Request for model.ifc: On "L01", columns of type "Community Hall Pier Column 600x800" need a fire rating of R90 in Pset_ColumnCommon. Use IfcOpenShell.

First a look at what the model holds.

```python
import ifcopenshell
import ifcopenshell.util.element

model = ifcopenshell.open("model.ifc")
print(model.schema)
storey = next(s for s in model.by_type("IfcBuildingStorey") if s.Name == "L01")
columns = [e for e in ifcopenshell.util.element.get_decomposition(storey) if e.is_a("IfcColumn")]
seen = {}
for e in columns:
    element_type = ifcopenshell.util.element.get_type(e)
    key = (element_type.Name if element_type != e and element_type else None, ifcopenshell.util.element.get_pset(e, "Pset_ColumnCommon", "FireRating"))
    seen[key] = seen.get(key, 0) + 1
for (name, value), count in sorted(seen.items(), key=str):
    print(count, "x", name, "|", value)
```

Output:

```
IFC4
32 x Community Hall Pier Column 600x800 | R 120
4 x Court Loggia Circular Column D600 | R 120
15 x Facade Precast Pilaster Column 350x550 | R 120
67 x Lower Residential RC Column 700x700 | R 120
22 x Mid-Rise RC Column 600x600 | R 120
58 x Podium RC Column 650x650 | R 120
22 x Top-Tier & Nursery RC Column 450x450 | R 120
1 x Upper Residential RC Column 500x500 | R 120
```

```python
import ifcopenshell
import ifcopenshell.api.pset
import ifcopenshell.util.element

model = ifcopenshell.open("model.ifc")

storey = next(s for s in model.by_type("IfcBuildingStorey") if s.Name == "L01")
columns = [e for e in ifcopenshell.util.element.get_decomposition(storey) if e.is_a("IfcColumn")]

count = 0
for e in columns:
    element_type = ifcopenshell.util.element.get_type(e)
    if element_type in (None, e) or element_type.Name != "Community Hall Pier Column 600x800":
        continue
    # add_pset returns the element's existing set when there is one.
    pset = ifcopenshell.api.pset.add_pset(model, product=e, name="Pset_ColumnCommon")
    ifcopenshell.api.pset.edit_pset(model, pset=pset, properties={"FireRating": "R90"})
    count += 1

print(count, "columns updated")

model.write("model_updated.ifc")
```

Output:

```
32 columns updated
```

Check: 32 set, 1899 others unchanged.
